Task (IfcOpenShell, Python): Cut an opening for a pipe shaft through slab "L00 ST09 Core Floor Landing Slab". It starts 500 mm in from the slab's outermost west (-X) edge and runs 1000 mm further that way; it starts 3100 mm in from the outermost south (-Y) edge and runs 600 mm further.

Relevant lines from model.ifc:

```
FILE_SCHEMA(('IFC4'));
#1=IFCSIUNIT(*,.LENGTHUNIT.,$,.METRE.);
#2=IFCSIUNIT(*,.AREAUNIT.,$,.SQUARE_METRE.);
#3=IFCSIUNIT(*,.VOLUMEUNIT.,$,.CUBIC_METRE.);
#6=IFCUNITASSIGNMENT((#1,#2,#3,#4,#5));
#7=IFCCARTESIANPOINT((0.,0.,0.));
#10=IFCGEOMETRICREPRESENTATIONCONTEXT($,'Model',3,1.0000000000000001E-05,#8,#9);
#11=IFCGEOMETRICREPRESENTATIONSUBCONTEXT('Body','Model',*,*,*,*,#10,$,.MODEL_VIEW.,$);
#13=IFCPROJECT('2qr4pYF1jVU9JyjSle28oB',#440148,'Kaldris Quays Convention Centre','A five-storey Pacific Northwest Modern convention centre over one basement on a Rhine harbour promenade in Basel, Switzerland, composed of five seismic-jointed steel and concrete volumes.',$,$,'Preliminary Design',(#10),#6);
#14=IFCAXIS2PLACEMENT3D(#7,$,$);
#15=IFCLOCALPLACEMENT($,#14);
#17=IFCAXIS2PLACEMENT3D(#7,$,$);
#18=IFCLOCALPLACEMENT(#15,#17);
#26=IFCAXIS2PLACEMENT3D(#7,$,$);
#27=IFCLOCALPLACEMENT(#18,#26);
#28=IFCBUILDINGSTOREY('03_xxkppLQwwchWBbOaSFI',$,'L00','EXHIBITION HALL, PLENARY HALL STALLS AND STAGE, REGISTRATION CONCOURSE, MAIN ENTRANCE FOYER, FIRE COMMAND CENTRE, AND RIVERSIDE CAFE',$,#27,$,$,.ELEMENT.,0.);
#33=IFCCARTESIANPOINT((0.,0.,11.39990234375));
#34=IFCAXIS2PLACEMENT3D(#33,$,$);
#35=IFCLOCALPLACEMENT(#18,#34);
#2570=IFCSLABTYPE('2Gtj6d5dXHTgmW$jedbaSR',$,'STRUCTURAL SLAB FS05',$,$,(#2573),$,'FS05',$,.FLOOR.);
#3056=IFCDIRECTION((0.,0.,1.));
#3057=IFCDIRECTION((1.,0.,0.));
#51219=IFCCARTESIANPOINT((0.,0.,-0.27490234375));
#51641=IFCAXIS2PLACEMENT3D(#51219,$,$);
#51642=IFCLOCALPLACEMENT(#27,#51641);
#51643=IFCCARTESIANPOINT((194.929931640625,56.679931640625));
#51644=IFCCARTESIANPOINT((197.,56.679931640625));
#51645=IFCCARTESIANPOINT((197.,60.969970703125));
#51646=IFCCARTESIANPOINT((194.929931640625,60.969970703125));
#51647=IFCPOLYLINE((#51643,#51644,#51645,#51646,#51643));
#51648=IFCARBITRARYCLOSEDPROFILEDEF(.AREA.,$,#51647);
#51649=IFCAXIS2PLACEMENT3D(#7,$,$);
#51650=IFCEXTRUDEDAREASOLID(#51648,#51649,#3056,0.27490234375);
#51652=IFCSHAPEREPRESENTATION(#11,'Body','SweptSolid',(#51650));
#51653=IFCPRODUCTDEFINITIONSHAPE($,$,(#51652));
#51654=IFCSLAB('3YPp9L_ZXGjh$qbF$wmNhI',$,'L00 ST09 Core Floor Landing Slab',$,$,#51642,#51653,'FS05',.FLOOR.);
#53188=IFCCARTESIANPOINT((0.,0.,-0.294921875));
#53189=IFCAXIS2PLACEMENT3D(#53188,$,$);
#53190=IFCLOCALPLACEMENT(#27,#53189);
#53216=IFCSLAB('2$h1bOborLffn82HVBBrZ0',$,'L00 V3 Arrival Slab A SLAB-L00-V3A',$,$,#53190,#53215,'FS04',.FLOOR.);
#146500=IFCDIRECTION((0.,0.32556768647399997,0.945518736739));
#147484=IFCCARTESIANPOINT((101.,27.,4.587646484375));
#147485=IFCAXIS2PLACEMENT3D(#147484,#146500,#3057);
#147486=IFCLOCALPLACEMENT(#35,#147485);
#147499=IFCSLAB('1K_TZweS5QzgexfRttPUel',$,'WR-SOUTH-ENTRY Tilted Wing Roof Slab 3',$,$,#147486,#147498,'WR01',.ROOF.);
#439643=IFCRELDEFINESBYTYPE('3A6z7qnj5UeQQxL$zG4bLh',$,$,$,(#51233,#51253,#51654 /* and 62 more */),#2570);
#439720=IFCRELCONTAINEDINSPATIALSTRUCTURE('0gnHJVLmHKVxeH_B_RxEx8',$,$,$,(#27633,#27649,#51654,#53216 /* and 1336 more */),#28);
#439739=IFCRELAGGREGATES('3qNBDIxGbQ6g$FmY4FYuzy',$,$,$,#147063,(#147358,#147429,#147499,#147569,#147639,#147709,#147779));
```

```python
import numpy as np
import ifcopenshell
import ifcopenshell.api.feature
import ifcopenshell.api.geometry
import ifcopenshell.api.root
import ifcopenshell.geom
import ifcopenshell.util.placement
import ifcopenshell.util.representation
import ifcopenshell.util.shape
import ifcopenshell.util.unit

model = ifcopenshell.open("model.ifc")
unit_scale = ifcopenshell.util.unit.calculate_unit_scale(model)
settings = ifcopenshell.geom.settings()


def volume(element):
    """Net volume in cubic metres, openings subtracted."""
    shape = ifcopenshell.geom.create_shape(settings, element)
    return ifcopenshell.util.shape.get_volume(shape.geometry)


slab = model.by_id(51654)
before = volume(slab)

# Extent in the slab's own axes, in metres. The edges named are its -X and -Y sides.
slab_shape = ifcopenshell.geom.create_shape(settings, slab)
vertices = ifcopenshell.util.shape.get_vertices(slab_shape.geometry)
x_min, y_min, bottom = vertices.min(axis=0)
top = vertices[:, 2].max()

opening = ifcopenshell.api.root.create_entity(model, ifc_class="IfcOpeningElement", name="Pipe shaft opening", predefined_type="OPENING")
context = ifcopenshell.util.representation.get_context(model, "Model", "Body", "MODEL_VIEW")
width, depth = 1, 0.6
outline = [(0.0, 0.0), (width, 0.0), (width, depth), (0.0, depth), (0.0, 0.0)]
# Overshoot both faces by 50 mm so the cut is clean.
shape = ifcopenshell.api.geometry.add_slab_representation(
    model, context=context, depth=top - bottom + 0.1, polyline=outline
)
ifcopenshell.api.geometry.assign_representation(model, product=opening, representation=shape)

matrix = ifcopenshell.util.placement.get_local_placement(slab.ObjectPlacement)
matrix[:, 3] = matrix @ np.append(np.array([x_min + 0.5, y_min + 3.1, bottom - 0.05]) / unit_scale, 1.0)
ifcopenshell.api.geometry.edit_object_placement(model, product=opening, matrix=matrix, is_si=False)
ifcopenshell.api.feature.add_feature(model, feature=opening, element=slab)

after = volume(slab)

print(f"slab volume {before:.3f} -> {after:.3f} m3")

model.write("model-out.ifc")
```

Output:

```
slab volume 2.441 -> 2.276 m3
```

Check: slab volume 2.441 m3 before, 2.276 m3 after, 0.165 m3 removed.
